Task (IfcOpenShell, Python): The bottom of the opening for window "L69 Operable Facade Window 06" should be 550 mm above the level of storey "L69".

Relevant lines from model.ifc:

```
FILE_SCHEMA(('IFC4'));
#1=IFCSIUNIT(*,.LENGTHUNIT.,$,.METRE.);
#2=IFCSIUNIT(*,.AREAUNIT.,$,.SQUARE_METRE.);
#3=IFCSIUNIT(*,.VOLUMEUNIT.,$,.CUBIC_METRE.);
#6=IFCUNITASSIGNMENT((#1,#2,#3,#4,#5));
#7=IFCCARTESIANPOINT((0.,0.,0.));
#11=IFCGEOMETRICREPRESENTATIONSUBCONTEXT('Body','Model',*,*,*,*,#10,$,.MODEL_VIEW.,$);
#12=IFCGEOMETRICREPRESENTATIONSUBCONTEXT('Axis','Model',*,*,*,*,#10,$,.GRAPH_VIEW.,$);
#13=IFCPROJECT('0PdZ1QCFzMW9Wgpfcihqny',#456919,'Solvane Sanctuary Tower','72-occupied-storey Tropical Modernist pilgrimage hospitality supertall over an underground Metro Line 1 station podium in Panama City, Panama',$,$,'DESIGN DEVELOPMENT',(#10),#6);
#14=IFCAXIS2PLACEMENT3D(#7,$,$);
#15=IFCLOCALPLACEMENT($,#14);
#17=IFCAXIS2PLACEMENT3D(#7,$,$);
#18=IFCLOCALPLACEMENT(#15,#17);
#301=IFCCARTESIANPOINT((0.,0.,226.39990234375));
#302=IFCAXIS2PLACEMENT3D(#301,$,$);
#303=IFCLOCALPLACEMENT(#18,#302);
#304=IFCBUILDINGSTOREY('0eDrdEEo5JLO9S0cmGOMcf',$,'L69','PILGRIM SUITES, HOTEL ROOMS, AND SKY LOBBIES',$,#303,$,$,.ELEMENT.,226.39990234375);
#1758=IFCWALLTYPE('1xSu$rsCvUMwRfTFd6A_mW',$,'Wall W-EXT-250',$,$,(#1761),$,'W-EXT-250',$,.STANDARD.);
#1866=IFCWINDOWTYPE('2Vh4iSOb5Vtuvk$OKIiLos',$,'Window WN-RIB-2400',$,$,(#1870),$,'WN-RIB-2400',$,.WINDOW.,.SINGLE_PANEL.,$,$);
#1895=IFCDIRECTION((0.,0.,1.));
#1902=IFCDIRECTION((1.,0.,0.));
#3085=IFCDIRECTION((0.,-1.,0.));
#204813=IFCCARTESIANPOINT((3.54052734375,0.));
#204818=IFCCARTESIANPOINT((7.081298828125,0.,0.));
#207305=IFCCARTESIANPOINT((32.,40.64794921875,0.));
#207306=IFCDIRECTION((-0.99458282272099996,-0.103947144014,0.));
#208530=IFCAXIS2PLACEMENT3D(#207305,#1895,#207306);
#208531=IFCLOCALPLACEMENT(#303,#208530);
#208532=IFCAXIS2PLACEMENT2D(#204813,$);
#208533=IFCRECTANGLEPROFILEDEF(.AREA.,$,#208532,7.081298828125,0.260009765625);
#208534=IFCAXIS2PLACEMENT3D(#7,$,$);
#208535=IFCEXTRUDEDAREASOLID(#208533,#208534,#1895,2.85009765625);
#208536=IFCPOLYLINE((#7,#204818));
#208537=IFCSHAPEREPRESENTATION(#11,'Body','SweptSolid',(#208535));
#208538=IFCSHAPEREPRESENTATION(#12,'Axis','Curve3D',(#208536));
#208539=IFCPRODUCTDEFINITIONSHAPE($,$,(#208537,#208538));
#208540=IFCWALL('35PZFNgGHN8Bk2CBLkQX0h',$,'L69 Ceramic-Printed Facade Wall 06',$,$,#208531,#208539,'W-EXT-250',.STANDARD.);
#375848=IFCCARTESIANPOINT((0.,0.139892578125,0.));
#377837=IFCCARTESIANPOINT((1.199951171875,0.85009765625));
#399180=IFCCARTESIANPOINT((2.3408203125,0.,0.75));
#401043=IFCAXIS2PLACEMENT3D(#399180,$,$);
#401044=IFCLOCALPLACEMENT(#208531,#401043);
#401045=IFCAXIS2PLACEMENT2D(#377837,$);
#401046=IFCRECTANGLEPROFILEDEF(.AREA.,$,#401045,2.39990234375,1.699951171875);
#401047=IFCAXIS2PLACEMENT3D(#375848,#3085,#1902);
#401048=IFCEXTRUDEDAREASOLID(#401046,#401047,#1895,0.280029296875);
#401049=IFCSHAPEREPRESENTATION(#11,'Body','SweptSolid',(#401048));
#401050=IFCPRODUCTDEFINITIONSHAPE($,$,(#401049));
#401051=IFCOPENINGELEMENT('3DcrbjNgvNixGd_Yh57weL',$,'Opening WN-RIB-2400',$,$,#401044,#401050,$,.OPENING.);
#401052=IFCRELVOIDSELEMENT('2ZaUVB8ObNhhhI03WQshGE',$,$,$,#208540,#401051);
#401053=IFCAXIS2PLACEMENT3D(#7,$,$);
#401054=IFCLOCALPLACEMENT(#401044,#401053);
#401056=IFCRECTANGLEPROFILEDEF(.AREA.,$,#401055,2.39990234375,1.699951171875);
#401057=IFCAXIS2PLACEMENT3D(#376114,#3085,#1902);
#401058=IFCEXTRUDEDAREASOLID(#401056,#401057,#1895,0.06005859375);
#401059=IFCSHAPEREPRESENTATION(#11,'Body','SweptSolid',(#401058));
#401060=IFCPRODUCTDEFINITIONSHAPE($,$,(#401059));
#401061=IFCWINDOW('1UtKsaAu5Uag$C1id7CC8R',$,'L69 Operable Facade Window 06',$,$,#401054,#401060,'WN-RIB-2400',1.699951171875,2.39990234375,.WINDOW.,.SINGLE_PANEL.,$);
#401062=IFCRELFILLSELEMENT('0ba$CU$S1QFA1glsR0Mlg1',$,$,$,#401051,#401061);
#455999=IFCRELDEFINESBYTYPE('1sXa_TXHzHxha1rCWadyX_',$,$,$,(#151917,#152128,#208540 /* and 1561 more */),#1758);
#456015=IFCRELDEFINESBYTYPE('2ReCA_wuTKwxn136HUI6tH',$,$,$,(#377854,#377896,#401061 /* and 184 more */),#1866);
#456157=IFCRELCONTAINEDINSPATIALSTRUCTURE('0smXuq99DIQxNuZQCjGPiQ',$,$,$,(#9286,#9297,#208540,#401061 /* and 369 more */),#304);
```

```python
import numpy as np
import ifcopenshell
import ifcopenshell.api.geometry
import ifcopenshell.geom
import ifcopenshell.util.element
import ifcopenshell.util.placement
import ifcopenshell.util.shape
import ifcopenshell.util.unit

model = ifcopenshell.open("model.ifc")
unit_scale = ifcopenshell.util.unit.calculate_unit_scale(model)

window = model.by_id(401061)
opening = window.FillsVoids[0].RelatingOpeningElement
storey = ifcopenshell.util.element.get_container(window, ifc_class="IfcBuildingStorey")
level = ifcopenshell.util.placement.get_local_placement(storey.ObjectPlacement)[2, 3]

# The opening's origin need not be at the sill, so measure its lowest point.
shape = ifcopenshell.geom.create_shape(ifcopenshell.geom.settings(), opening)
bottom = ifcopenshell.util.shape.get_shape_bottom_elevation(shape, shape.geometry) / unit_scale
dz = level + 0.55 / unit_scale - bottom

shift = np.array([0.0, 0.0, dz])
# The window is placed relative to its opening, so it follows when the opening moves.
matrix = ifcopenshell.util.placement.get_local_placement(opening.ObjectPlacement)
matrix[:3, 3] += shift
ifcopenshell.api.geometry.edit_object_placement(
    model, product=opening, matrix=matrix, is_si=False, should_transform_children=True
)

print(f"moved by {dz * unit_scale:+.3f} m")

model.write("model_rev.ifc")
```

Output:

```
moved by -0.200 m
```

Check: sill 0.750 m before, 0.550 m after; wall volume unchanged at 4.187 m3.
